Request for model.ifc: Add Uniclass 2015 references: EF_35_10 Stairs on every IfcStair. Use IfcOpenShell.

First a look at what the model holds.

```python
import ifcopenshell

model = ifcopenshell.open("model.ifc")
print(model.schema)
print("classifications:", [c.Name for c in model.by_type("IfcClassification")])
for ifc_class in ("IfcDoor", "IfcRoof", "IfcStair", "IfcWall", "IfcWindow"):
    print(ifc_class, len(model.by_type(ifc_class)))
```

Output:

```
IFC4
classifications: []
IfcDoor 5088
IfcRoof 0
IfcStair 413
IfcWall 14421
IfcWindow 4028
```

```python
import ifcopenshell
import ifcopenshell.api.classification

model = ifcopenshell.open("model.ifc")

system = ifcopenshell.api.classification.add_classification(model, classification="Uniclass 2015")

codes = {
    "IfcStair": ("EF_35_10", "Stairs"),
}
for ifc_class, (code, name) in codes.items():
    products = model.by_type(ifc_class)
    ifcopenshell.api.classification.add_reference(
        model, products=products, classification=system, identification=code, name=name
    )
    print(code, len(products))

model.write("model_updated.ifc")
```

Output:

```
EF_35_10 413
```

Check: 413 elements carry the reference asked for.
